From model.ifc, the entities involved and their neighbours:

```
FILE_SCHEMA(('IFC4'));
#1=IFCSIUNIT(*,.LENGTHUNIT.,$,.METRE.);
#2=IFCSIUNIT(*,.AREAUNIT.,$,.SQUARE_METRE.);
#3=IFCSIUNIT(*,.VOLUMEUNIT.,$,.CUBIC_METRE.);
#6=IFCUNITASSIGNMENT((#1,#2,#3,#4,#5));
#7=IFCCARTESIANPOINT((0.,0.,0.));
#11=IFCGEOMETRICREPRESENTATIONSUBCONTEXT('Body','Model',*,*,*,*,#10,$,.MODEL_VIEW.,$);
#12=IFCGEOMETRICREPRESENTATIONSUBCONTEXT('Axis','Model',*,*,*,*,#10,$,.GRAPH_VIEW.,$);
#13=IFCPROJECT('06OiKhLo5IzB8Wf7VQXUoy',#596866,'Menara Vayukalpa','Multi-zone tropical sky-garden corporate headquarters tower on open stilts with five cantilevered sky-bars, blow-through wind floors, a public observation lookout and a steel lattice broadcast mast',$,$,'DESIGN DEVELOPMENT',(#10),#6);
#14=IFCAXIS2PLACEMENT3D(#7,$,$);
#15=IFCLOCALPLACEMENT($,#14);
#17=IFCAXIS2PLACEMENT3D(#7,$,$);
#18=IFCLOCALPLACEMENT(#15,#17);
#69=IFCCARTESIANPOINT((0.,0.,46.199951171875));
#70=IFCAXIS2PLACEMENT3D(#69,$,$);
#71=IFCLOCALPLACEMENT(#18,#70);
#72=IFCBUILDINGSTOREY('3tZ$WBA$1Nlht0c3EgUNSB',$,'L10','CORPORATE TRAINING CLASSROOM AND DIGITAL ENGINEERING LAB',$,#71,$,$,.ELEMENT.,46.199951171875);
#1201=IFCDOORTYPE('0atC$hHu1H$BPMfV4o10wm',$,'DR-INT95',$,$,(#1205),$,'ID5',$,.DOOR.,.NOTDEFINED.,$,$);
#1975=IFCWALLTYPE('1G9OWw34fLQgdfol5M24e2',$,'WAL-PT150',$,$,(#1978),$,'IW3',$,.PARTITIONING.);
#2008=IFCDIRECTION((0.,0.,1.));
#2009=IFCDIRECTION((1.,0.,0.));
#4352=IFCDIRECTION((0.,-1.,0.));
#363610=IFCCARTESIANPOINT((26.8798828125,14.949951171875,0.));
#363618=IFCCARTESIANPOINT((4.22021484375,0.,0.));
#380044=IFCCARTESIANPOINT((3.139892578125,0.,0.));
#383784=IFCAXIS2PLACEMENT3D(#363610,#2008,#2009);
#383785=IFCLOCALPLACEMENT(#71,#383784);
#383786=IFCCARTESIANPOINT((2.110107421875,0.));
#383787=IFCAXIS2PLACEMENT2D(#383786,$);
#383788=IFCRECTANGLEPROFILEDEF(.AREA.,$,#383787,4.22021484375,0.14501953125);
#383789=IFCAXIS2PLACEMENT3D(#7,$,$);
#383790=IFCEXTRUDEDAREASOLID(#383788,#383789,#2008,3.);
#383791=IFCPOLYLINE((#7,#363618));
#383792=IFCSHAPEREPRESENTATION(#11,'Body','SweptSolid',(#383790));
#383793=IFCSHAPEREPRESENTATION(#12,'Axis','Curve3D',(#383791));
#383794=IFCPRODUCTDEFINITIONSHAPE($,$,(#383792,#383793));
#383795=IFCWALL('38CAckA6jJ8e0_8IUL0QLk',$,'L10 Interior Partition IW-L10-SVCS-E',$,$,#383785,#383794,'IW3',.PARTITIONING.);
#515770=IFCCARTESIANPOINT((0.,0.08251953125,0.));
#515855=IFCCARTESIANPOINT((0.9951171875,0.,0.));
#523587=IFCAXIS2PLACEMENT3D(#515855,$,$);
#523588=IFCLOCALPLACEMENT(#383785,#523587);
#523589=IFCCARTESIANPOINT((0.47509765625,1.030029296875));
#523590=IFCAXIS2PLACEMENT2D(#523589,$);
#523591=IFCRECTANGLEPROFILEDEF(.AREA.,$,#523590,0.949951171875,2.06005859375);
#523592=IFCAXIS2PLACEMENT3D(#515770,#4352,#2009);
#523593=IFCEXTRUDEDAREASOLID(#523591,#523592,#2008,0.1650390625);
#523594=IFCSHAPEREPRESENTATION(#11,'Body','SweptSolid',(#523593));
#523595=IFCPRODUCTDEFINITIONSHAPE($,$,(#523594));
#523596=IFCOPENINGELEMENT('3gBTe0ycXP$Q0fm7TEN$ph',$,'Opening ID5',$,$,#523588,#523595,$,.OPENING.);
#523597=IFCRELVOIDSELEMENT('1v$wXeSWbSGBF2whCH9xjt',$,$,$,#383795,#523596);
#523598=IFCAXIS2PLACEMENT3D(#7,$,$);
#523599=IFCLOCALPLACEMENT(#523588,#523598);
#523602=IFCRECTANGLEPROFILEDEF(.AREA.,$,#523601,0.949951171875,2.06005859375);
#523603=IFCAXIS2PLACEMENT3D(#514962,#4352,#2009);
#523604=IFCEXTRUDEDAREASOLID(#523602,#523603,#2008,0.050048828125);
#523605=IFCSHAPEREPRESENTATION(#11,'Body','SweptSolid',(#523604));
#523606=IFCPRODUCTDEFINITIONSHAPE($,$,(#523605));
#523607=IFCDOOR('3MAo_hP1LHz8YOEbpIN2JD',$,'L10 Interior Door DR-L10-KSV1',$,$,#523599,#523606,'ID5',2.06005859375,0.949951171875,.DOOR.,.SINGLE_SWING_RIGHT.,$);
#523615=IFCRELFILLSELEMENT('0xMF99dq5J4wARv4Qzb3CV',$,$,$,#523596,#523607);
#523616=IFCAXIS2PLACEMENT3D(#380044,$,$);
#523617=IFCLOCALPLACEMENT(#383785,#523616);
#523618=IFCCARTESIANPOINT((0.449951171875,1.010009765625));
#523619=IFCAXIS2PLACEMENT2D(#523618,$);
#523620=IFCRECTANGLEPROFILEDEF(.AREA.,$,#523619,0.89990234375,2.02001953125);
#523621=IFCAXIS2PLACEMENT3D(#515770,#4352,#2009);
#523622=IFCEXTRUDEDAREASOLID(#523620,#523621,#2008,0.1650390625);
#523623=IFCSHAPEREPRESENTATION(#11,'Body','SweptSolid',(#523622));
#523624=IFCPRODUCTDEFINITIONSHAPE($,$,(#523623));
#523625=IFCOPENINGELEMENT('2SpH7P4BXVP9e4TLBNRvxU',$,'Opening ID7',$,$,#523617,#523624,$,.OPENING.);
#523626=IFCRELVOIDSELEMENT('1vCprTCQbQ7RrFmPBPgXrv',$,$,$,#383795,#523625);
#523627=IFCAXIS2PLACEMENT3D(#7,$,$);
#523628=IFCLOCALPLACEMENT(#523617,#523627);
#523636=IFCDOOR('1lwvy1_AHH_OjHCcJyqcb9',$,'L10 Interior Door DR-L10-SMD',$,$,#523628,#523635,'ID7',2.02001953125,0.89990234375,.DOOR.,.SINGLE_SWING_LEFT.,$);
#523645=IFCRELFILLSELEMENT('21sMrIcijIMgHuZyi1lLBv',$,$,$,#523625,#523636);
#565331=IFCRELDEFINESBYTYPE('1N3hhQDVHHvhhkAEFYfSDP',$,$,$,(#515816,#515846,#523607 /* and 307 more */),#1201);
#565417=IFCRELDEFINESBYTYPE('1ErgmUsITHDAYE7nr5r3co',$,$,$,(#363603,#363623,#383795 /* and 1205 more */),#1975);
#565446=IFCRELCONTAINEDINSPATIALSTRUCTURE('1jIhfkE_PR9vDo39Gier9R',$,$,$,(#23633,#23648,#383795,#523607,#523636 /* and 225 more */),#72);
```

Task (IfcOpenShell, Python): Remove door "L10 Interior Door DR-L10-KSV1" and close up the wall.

```python
import ifcopenshell
import ifcopenshell.api.feature
import ifcopenshell.api.root
import ifcopenshell.geom
import ifcopenshell.util.shape

model = ifcopenshell.open("model.ifc")
settings = ifcopenshell.geom.settings()


def volume(element):
    """Net volume in cubic metres, openings subtracted."""
    shape = ifcopenshell.geom.create_shape(settings, element)
    return ifcopenshell.util.shape.get_volume(shape.geometry)


door = model.by_guid("3MAo_hP1LHz8YOEbpIN2JD")
opening = door.FillsVoids[0].RelatingOpeningElement
wall = opening.VoidsElements[0].RelatingBuildingElement
before = volume(wall)

ifcopenshell.api.root.remove_product(model, product=door)
ifcopenshell.api.feature.remove_feature(model, feature=opening)

after = volume(wall)

print(f"wall volume {before:.3f} -> {after:.3f} m3")

model.write("model_v2.ifc")
```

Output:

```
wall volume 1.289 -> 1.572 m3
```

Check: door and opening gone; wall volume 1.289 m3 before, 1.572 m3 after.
